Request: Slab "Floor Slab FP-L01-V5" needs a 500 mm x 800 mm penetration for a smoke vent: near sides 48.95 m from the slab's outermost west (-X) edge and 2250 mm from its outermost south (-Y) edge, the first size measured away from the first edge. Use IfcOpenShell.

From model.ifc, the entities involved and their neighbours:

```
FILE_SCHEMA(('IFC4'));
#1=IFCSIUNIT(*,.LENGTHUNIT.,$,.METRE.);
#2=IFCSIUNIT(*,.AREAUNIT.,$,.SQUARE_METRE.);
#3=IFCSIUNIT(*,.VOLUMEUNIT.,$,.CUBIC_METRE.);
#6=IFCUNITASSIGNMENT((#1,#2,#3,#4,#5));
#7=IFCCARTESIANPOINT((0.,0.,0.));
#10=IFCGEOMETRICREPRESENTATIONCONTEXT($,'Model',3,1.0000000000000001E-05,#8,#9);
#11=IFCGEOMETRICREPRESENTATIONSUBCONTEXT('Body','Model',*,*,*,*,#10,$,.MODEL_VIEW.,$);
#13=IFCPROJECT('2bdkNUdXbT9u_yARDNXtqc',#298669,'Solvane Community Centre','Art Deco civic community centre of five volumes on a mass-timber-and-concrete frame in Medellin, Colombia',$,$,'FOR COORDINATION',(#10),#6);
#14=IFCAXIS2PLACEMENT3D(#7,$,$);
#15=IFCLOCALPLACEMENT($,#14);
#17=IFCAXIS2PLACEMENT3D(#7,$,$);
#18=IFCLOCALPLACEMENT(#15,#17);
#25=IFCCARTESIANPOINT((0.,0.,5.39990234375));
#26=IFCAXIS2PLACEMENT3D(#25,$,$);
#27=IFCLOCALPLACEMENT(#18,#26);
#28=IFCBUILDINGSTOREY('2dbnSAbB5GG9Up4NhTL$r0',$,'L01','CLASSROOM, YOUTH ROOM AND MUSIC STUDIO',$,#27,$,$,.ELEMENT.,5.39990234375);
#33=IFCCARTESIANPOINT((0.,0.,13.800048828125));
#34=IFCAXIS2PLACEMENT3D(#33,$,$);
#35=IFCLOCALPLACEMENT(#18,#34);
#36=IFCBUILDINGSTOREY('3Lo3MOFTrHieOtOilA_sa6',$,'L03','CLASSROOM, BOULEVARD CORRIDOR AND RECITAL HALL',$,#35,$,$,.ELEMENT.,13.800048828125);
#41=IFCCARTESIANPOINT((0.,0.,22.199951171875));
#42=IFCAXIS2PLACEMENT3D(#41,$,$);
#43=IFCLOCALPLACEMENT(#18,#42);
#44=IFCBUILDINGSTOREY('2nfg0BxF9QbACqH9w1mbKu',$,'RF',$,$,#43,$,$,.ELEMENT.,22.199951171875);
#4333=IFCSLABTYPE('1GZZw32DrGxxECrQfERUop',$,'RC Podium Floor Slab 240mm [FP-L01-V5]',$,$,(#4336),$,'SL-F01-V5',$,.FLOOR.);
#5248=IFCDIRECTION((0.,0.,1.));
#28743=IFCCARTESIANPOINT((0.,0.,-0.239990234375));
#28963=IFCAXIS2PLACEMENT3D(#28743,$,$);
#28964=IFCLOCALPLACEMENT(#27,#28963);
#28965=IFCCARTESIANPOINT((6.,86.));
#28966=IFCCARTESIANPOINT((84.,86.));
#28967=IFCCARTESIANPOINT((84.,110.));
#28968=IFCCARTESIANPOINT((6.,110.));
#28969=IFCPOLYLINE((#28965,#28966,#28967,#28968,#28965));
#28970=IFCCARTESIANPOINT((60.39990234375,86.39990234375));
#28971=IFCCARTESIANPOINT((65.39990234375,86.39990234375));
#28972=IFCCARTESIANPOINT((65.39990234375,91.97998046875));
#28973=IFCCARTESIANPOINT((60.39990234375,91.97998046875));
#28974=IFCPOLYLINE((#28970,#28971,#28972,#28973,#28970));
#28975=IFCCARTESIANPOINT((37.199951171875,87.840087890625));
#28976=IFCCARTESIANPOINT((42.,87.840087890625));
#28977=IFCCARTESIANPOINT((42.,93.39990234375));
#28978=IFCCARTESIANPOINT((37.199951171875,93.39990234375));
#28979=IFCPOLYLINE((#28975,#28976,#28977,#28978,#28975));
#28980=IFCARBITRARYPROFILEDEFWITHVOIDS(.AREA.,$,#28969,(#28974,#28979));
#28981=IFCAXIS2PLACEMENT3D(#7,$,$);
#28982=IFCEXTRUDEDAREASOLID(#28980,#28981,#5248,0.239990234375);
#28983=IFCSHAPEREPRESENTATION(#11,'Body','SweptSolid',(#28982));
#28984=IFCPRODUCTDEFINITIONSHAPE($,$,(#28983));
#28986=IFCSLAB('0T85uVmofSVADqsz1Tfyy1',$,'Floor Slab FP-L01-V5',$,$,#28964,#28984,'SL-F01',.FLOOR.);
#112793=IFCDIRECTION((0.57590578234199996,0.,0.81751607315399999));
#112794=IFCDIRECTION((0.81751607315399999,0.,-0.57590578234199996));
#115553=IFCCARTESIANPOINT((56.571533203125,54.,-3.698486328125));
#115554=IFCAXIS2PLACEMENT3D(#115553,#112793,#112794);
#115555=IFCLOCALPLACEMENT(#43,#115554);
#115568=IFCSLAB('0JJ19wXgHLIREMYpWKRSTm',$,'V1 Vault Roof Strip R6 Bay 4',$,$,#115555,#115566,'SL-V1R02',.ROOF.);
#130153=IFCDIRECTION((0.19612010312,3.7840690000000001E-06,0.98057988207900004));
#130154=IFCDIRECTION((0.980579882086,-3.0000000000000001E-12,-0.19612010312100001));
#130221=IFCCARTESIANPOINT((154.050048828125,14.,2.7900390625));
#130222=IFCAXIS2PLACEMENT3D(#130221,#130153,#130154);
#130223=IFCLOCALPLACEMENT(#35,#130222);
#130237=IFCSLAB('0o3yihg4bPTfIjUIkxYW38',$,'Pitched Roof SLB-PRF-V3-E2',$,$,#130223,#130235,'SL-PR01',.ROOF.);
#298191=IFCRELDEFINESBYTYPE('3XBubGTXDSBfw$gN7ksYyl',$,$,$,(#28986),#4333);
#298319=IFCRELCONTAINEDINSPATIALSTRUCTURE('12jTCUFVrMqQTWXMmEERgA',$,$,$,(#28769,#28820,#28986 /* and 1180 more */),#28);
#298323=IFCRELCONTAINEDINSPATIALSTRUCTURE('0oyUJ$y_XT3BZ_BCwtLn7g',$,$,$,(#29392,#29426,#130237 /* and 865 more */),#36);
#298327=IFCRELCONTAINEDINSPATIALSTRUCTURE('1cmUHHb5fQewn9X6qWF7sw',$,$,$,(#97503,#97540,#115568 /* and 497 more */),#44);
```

```python
import numpy as np
import ifcopenshell
import ifcopenshell.api.feature
import ifcopenshell.api.geometry
import ifcopenshell.api.root
import ifcopenshell.geom
import ifcopenshell.util.placement
import ifcopenshell.util.representation
import ifcopenshell.util.shape
import ifcopenshell.util.unit

model = ifcopenshell.open("model.ifc")
unit_scale = ifcopenshell.util.unit.calculate_unit_scale(model)
settings = ifcopenshell.geom.settings()


def volume(element):
    """Net volume in cubic metres, openings subtracted."""
    shape = ifcopenshell.geom.create_shape(settings, element)
    return ifcopenshell.util.shape.get_volume(shape.geometry)


slab = model.by_id(28986)
before = volume(slab)

# Extent in the slab's own axes, in metres. The edges named are its -X and -Y sides.
slab_shape = ifcopenshell.geom.create_shape(settings, slab)
vertices = ifcopenshell.util.shape.get_vertices(slab_shape.geometry)
x_min, y_min, bottom = vertices.min(axis=0)
top = vertices[:, 2].max()

opening = ifcopenshell.api.root.create_entity(model, ifc_class="IfcOpeningElement", name="Smoke vent opening", predefined_type="OPENING")
context = ifcopenshell.util.representation.get_context(model, "Model", "Body", "MODEL_VIEW")
width, depth = 0.5, 0.8
outline = [(0.0, 0.0), (width, 0.0), (width, depth), (0.0, depth), (0.0, 0.0)]
# Overshoot both faces by 50 mm so the cut is clean.
shape = ifcopenshell.api.geometry.add_slab_representation(
    model, context=context, depth=top - bottom + 0.1, polyline=outline
)
ifcopenshell.api.geometry.assign_representation(model, product=opening, representation=shape)

matrix = ifcopenshell.util.placement.get_local_placement(slab.ObjectPlacement)
matrix[:, 3] = matrix @ np.append(np.array([x_min + 48.95, y_min + 2.25, bottom - 0.05]) / unit_scale, 1.0)
ifcopenshell.api.geometry.edit_object_placement(model, product=opening, matrix=matrix, is_si=False)
ifcopenshell.api.feature.add_feature(model, feature=opening, element=slab)

after = volume(slab)

print(f"slab volume {before:.3f} -> {after:.3f} m3")

model.write("model_updated.ifc")
```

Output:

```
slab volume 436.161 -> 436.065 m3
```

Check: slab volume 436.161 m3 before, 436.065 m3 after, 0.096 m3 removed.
